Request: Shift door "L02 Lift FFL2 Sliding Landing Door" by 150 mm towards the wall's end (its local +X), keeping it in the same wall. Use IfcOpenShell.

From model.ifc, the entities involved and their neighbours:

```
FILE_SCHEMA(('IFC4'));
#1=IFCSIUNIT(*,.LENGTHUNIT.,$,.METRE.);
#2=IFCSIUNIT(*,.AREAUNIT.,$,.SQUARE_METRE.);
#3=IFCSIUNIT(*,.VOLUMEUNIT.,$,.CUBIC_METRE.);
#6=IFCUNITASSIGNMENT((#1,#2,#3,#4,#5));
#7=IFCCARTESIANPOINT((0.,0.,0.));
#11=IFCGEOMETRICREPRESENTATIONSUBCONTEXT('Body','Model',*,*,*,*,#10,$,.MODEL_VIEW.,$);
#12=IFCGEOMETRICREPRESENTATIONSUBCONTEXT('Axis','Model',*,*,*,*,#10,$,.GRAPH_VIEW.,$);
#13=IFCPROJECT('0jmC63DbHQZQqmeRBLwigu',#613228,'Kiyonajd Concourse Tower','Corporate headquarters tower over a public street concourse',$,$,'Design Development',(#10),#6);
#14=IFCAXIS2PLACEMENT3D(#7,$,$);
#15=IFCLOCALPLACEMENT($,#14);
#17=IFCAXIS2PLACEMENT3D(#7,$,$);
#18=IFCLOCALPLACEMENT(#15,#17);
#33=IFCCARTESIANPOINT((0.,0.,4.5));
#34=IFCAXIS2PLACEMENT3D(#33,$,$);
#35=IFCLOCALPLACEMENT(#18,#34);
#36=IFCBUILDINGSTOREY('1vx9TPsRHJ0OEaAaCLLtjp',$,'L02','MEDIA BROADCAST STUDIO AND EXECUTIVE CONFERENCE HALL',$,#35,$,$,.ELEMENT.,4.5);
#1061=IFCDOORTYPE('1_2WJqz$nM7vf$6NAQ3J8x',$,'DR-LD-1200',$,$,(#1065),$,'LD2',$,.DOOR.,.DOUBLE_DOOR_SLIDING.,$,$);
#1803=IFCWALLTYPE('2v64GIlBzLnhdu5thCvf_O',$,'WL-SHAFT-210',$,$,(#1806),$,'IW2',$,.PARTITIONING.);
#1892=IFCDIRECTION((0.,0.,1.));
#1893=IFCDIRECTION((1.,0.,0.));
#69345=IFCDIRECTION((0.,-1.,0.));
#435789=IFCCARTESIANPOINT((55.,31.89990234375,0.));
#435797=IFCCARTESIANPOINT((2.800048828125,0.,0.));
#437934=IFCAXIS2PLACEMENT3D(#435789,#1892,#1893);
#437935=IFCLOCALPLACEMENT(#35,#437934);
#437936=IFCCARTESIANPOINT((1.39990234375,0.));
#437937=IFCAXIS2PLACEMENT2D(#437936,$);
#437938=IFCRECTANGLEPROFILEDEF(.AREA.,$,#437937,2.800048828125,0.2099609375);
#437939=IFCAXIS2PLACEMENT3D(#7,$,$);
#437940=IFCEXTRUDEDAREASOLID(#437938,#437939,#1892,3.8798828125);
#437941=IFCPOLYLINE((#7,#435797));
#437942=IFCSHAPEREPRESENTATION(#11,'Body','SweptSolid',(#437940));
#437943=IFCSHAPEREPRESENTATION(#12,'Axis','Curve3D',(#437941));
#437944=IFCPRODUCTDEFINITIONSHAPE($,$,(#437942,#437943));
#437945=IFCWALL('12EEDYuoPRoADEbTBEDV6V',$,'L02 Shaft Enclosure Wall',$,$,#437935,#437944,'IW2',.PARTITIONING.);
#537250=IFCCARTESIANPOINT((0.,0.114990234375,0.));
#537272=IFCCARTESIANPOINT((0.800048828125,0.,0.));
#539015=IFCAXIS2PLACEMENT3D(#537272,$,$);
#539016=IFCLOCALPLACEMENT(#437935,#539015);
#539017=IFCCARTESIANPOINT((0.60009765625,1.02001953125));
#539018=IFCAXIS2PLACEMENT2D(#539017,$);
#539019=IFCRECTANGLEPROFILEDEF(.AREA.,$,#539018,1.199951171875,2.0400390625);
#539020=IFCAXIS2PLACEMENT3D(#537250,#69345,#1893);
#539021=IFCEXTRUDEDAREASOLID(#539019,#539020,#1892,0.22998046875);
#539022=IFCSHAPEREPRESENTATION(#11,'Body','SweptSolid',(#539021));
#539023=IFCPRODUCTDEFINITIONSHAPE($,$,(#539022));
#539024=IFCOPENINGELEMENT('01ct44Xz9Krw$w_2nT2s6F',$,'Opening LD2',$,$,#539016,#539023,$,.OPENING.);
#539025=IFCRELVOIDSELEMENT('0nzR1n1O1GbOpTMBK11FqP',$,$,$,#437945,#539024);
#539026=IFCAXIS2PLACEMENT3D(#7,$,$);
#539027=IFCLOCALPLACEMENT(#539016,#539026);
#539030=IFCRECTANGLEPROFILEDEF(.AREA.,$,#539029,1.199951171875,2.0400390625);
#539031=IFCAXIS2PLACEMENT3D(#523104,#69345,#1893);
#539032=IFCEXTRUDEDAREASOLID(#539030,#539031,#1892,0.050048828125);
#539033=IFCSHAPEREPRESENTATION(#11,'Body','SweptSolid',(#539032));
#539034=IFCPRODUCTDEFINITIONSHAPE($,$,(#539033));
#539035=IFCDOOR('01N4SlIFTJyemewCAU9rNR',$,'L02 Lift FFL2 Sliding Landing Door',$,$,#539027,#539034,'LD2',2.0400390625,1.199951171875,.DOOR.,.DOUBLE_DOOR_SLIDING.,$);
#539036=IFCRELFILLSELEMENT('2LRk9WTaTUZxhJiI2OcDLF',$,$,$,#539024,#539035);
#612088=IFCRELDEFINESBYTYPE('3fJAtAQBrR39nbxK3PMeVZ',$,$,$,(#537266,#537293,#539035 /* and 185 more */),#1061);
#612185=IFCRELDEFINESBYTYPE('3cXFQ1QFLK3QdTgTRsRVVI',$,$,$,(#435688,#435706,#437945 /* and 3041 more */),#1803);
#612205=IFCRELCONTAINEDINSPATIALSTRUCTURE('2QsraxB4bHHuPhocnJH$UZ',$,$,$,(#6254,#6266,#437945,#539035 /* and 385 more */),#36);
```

```python
import ifcopenshell
import ifcopenshell.api.geometry
import ifcopenshell.util.placement

model = ifcopenshell.open("model.ifc")

door = model.by_guid("01N4SlIFTJyemewCAU9rNR")
opening = door.FillsVoids[0].RelatingOpeningElement
wall = opening.VoidsElements[0].RelatingBuildingElement

wall_matrix = ifcopenshell.util.placement.get_local_placement(wall.ObjectPlacement)
shift = wall_matrix[:3, 0] * 0.15
before = ifcopenshell.util.placement.get_local_placement(door.ObjectPlacement)[:3, 3].copy()

# The door is placed relative to its opening, so it follows when the opening moves.
matrix = ifcopenshell.util.placement.get_local_placement(opening.ObjectPlacement)
matrix[:3, 3] += shift
ifcopenshell.api.geometry.edit_object_placement(
    model, product=opening, matrix=matrix, is_si=False, should_transform_children=True
)

after = ifcopenshell.util.placement.get_local_placement(door.ObjectPlacement)[:3, 3]
print("door moved by", (after - before).round(3) + 0.0)

model.write("model-out.ifc")
```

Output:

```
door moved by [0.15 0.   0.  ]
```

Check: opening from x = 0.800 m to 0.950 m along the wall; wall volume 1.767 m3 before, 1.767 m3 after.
